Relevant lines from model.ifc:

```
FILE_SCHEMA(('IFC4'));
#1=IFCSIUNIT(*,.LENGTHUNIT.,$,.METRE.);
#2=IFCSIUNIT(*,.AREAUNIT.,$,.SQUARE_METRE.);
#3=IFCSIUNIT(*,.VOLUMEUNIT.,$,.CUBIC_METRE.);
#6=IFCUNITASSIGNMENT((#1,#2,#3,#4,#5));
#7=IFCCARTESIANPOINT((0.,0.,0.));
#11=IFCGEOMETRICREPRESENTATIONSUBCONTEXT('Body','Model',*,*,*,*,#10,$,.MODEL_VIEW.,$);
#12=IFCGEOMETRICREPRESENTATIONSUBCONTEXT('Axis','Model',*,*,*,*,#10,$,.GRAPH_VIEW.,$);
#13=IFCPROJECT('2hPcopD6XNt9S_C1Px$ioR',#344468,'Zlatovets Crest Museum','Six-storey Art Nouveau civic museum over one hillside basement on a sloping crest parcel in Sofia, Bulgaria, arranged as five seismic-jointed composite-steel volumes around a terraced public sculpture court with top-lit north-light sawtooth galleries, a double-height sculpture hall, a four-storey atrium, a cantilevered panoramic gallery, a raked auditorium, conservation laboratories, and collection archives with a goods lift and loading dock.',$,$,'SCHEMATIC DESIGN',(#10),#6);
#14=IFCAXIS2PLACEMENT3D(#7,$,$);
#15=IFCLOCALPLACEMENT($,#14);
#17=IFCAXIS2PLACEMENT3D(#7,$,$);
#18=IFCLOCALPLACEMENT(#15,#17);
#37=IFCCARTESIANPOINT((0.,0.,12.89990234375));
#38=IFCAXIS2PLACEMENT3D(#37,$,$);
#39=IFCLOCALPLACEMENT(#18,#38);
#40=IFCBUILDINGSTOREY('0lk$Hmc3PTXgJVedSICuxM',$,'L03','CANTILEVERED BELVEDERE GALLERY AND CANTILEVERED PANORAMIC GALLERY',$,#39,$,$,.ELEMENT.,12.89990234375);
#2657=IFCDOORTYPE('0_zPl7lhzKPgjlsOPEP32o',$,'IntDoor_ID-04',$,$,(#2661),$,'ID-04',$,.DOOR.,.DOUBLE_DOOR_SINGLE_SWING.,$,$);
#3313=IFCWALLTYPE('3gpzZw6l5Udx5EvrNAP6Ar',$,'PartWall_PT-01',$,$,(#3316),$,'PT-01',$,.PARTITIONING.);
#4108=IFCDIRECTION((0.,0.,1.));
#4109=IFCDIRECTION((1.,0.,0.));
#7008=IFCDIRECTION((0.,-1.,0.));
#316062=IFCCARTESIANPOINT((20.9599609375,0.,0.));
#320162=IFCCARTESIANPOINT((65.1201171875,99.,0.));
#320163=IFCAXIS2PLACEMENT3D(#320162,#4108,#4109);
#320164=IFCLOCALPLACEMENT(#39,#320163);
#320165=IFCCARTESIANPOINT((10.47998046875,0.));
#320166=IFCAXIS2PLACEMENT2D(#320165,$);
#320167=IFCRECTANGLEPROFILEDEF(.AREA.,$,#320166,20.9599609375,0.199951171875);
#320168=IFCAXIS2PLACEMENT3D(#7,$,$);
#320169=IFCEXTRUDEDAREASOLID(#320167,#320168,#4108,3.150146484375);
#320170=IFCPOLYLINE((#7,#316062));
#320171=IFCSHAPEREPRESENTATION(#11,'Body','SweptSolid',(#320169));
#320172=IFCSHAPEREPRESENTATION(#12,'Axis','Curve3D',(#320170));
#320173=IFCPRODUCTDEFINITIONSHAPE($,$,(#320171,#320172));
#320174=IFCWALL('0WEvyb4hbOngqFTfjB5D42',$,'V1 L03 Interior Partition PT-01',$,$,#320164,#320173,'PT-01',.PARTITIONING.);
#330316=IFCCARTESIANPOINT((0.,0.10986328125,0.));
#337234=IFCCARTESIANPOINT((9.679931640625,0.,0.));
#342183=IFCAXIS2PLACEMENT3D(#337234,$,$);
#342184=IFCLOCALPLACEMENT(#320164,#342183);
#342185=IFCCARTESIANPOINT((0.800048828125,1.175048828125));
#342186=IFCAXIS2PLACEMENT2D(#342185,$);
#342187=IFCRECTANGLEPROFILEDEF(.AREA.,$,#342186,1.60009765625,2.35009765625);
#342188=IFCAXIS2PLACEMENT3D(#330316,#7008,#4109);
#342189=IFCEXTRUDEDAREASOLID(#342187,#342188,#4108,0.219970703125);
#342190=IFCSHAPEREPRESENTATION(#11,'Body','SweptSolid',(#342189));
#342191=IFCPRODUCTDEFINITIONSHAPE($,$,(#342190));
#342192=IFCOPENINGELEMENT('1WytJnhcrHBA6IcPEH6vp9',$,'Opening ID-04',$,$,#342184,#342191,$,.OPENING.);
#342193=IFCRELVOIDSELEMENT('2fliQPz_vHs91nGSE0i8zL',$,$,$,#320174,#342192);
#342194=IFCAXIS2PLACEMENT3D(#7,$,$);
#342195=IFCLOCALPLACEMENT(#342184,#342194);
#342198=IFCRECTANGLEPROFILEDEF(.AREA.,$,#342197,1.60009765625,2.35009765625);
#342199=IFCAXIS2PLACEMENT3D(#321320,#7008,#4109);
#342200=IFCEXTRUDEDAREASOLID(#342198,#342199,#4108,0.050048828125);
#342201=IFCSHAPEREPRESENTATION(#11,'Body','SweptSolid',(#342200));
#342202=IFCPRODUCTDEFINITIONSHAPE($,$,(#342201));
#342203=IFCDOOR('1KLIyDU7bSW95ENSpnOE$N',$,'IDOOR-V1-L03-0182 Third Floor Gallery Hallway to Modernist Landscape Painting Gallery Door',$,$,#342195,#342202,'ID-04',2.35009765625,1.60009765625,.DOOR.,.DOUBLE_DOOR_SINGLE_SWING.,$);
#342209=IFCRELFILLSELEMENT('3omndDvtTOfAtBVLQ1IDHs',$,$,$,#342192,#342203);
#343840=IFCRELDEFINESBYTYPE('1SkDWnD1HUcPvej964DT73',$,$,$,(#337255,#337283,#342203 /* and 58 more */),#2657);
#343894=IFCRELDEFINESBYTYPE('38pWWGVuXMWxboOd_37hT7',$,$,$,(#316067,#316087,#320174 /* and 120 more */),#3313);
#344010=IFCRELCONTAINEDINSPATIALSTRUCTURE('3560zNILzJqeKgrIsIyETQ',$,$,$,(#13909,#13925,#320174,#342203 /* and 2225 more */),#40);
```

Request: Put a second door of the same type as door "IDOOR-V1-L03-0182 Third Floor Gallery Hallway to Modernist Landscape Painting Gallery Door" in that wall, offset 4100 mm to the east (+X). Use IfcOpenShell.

```python
import ifcopenshell
import ifcopenshell.api.feature
import ifcopenshell.api.geometry
import ifcopenshell.api.root
import ifcopenshell.geom
import ifcopenshell.util.element
import ifcopenshell.util.placement
import ifcopenshell.util.shape
import ifcopenshell.util.unit

model = ifcopenshell.open("model.ifc")
unit_scale = ifcopenshell.util.unit.calculate_unit_scale(model)
settings = ifcopenshell.geom.settings()


def volume(element):
    """Net volume in cubic metres, openings subtracted."""
    shape = ifcopenshell.geom.create_shape(settings, element)
    return ifcopenshell.util.shape.get_volume(shape.geometry)


door = model.by_guid("1KLIyDU7bSW95ENSpnOE$N")
opening = door.FillsVoids[0].RelatingOpeningElement
wall = opening.VoidsElements[0].RelatingBuildingElement
before = volume(wall)
shift = ifcopenshell.util.placement.get_local_placement(wall.ObjectPlacement)[:3, 0] * 4.1 / unit_scale

# copy_class copies the void relationship, type, container and properties, but no geometry.
new_opening = ifcopenshell.api.root.copy_class(model, product=opening)
new_opening.Representation = ifcopenshell.util.element.copy_deep(
    model, opening.Representation, exclude=["IfcGeometricRepresentationContext", "IfcRepresentationMap"]
)
new_door = ifcopenshell.api.root.copy_class(model, product=door)
new_door.Representation = ifcopenshell.util.element.copy_deep(
    model, door.Representation, exclude=["IfcGeometricRepresentationContext", "IfcRepresentationMap"]
)
new_door.Tag = None
ifcopenshell.api.feature.add_filling(model, opening=new_opening, element=new_door)

for old, new in ((opening, new_opening), (door, new_door)):
    matrix = ifcopenshell.util.placement.get_local_placement(old.ObjectPlacement)
    matrix[:3, 3] += shift
    ifcopenshell.api.geometry.edit_object_placement(model, product=new, matrix=matrix, is_si=False)

after = volume(wall)

print(f"wall volume {before:.3f} -> {after:.3f} m3")

model.write("model_edited.ifc")
```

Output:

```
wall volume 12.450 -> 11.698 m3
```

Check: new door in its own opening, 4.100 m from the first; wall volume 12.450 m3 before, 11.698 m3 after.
